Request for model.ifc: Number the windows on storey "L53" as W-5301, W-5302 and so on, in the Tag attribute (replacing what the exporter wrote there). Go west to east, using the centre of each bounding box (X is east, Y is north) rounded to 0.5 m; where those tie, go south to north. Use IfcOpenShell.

First a look at what the model holds.

```python
import ifcopenshell
import ifcopenshell.util.element
import ifcopenshell.util.placement

model = ifcopenshell.open("model.ifc")
print(model.schema)
storey = next(s for s in model.by_type("IfcBuildingStorey") if s.Name == "L53")
windows = [e for e in ifcopenshell.util.element.get_decomposition(storey) if e.is_a("IfcWindow")]
for e in sorted(windows, key=lambda e: e.id()):
    origin = ifcopenshell.util.placement.get_local_placement(e.ObjectPlacement)[:3, 3]
    print(e.id(), e.Tag, e.Name, origin.round(2) + 0.0, sep=" | ")
```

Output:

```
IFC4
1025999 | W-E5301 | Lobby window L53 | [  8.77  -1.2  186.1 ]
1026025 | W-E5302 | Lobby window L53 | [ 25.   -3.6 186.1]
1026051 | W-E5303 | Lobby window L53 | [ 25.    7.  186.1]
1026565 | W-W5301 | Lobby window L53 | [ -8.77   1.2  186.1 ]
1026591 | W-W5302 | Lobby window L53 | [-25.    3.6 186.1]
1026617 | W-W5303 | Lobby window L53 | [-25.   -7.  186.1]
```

```python
import ifcopenshell
import ifcopenshell.geom
import ifcopenshell.util.element
import ifcopenshell.util.shape

model = ifcopenshell.open("model.ifc")
settings = ifcopenshell.geom.settings()
settings.set("use-world-coords", True)


def centre(element):
    shape = ifcopenshell.geom.create_shape(settings, element)
    return ifcopenshell.util.shape.get_bbox_centroid(shape.geometry)


storey = next(s for s in model.by_type("IfcBuildingStorey") if s.Name == "L53")
windows = [e for e in ifcopenshell.util.element.get_decomposition(storey) if e.is_a("IfcWindow")]

# Insertion points can sit at a corner or the storey origin, so sort by the geometry (in metres).
centres = {e: centre(e) for e in windows}
windows.sort(key=lambda e: (round(centres[e][0] / 0.5), centres[e][1]))

for i, e in enumerate(windows, start=1):
    number = f"W-53{i:02d}"
    e.Tag = number
    print(e.id(), number)

model.write("model_v2.ifc")
```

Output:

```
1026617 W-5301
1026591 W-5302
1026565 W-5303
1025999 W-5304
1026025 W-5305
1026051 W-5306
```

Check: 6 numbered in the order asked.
